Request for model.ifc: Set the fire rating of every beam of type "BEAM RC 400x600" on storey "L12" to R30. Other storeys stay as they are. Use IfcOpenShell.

First a look at what the model holds.

```python
import ifcopenshell
import ifcopenshell.util.element

model = ifcopenshell.open("model.ifc")
print(model.schema)
storey = next(s for s in model.by_type("IfcBuildingStorey") if s.Name == "L12")
beams = [e for e in ifcopenshell.util.element.get_decomposition(storey) if e.is_a("IfcBeam")]
seen = {}
for e in beams:
    element_type = ifcopenshell.util.element.get_type(e)
    key = (element_type.Name if element_type != e and element_type else None, ifcopenshell.util.element.get_pset(e, "Pset_BeamCommon", "FireRating"))
    seen[key] = seen.get(key, 0) + 1
for (name, value), count in sorted(seen.items(), key=str):
    print(count, "x", name, "|", value)
```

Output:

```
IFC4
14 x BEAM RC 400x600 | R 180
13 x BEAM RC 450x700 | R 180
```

```python
import ifcopenshell
import ifcopenshell.api.pset
import ifcopenshell.util.element

model = ifcopenshell.open("model.ifc")

storey = next(s for s in model.by_type("IfcBuildingStorey") if s.Name == "L12")
beams = [e for e in ifcopenshell.util.element.get_decomposition(storey) if e.is_a("IfcBeam")]

count = 0
for e in beams:
    element_type = ifcopenshell.util.element.get_type(e)
    if element_type in (None, e) or element_type.Name != "BEAM RC 400x600":
        continue
    # add_pset returns the element's existing set when there is one.
    pset = ifcopenshell.api.pset.add_pset(model, product=e, name="Pset_BeamCommon")
    ifcopenshell.api.pset.edit_pset(model, pset=pset, properties={"FireRating": "R30"})
    count += 1

print(count, "beams updated")

model.write("model-out.ifc")
```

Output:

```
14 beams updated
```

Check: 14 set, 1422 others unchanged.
